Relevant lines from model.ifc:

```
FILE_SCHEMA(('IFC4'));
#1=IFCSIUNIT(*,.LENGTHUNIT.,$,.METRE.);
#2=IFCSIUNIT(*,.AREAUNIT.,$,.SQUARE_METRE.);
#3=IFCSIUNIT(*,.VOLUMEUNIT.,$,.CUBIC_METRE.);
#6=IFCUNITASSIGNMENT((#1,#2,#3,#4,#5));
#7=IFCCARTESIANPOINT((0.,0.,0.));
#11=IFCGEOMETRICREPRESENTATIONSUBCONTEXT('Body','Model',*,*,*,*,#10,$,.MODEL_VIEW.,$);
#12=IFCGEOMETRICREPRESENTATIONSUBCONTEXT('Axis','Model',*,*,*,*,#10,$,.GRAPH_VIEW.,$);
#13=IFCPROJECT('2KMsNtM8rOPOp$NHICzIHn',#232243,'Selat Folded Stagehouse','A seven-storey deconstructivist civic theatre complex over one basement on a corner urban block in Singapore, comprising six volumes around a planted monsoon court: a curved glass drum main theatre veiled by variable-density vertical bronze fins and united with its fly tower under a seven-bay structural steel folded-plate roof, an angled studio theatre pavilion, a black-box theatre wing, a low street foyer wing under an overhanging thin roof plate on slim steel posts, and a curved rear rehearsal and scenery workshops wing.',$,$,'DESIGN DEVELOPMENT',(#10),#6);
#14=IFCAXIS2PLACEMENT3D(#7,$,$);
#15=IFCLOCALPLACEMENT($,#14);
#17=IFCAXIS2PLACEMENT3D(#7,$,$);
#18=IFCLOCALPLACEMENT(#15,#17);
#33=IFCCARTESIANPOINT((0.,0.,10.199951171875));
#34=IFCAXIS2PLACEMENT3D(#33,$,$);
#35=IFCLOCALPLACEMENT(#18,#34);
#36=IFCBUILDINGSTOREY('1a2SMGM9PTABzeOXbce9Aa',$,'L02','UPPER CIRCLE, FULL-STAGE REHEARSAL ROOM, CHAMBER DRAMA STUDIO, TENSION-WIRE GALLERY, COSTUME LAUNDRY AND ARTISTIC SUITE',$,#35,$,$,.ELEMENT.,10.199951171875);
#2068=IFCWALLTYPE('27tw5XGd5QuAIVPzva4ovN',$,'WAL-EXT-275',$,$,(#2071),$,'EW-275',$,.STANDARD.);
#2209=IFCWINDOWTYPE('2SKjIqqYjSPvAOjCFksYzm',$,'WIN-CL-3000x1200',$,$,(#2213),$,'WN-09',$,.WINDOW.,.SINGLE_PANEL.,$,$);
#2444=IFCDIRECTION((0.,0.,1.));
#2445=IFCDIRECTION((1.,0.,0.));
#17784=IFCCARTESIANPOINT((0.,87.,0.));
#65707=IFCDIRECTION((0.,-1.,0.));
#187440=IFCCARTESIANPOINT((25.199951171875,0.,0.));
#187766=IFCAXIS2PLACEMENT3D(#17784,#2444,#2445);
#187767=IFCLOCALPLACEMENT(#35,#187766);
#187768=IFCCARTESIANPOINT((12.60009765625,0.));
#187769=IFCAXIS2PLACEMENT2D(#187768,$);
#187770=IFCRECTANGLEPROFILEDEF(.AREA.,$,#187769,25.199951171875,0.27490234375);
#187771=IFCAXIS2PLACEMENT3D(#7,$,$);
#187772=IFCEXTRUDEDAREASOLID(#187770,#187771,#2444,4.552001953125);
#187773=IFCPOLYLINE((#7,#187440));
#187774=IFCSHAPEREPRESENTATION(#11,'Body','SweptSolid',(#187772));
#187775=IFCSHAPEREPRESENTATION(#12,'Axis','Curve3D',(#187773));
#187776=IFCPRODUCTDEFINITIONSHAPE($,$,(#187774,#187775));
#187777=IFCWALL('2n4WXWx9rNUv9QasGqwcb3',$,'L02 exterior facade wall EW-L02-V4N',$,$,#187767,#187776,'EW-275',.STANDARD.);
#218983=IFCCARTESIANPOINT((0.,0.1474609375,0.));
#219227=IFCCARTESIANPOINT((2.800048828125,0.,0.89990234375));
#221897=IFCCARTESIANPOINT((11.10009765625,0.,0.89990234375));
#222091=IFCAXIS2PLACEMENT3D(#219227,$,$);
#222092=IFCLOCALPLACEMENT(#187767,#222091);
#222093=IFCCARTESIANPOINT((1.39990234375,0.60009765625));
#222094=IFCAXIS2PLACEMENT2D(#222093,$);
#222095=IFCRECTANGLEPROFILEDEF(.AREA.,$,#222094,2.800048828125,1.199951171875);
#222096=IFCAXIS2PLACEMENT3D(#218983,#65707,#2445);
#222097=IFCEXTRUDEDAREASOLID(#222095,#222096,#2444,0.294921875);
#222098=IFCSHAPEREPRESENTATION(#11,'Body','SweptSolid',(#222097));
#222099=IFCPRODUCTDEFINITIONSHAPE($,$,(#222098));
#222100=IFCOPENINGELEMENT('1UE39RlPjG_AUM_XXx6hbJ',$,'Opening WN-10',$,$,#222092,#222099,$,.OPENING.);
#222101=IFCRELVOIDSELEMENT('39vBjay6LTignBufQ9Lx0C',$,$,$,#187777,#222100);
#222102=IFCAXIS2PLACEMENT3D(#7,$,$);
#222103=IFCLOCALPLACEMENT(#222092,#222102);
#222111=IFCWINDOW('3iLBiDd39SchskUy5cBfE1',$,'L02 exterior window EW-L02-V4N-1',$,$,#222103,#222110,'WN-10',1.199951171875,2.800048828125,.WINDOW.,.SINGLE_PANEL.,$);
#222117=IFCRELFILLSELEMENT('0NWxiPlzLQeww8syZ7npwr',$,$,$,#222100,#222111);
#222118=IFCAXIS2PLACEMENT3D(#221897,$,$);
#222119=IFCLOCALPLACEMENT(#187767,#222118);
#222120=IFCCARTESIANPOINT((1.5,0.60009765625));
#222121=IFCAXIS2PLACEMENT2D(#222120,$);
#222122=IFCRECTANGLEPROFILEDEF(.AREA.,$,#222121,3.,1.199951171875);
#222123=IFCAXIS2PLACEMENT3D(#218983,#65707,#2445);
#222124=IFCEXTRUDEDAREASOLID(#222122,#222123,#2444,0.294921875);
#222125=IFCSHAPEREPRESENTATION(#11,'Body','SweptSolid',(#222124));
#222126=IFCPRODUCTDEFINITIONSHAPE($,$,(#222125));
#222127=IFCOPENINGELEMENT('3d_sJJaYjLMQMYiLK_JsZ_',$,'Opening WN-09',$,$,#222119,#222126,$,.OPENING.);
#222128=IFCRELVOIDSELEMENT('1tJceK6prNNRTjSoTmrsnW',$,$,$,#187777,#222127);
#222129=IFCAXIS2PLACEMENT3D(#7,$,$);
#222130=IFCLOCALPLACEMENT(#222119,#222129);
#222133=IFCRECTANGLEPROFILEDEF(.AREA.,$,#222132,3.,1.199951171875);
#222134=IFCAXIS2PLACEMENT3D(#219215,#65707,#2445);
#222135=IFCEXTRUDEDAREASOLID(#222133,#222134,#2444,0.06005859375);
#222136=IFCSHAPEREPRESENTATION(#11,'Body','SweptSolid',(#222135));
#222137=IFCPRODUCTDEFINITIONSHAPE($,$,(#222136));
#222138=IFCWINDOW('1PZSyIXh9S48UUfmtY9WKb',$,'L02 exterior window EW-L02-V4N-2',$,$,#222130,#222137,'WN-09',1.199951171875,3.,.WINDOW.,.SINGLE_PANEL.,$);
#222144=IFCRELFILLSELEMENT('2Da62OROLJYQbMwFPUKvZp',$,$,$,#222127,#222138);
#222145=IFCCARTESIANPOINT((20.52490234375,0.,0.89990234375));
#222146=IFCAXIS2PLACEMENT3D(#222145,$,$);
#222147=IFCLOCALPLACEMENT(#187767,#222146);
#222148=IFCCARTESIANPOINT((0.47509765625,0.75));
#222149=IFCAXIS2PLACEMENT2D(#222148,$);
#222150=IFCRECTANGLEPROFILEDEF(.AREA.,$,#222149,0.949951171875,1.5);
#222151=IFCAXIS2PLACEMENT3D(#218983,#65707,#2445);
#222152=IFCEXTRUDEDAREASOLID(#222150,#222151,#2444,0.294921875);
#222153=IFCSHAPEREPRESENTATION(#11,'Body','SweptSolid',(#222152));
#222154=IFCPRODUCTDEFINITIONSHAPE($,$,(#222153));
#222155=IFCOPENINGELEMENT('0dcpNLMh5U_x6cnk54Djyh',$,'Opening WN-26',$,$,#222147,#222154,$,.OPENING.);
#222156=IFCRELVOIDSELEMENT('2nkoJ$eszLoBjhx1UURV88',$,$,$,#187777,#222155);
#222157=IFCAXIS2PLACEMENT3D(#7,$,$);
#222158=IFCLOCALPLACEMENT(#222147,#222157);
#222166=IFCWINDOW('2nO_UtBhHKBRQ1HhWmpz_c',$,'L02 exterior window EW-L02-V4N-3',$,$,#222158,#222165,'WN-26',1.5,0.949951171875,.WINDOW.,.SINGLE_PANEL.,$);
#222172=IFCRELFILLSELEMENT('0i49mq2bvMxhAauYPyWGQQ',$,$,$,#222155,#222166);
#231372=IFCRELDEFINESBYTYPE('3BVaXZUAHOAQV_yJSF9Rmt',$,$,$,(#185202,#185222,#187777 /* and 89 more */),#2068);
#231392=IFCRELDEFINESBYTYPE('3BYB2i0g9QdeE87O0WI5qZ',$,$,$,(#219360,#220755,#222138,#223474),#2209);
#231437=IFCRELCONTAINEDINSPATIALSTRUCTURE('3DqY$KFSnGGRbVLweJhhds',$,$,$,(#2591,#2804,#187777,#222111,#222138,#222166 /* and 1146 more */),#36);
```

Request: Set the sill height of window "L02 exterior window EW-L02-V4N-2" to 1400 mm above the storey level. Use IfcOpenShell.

```python
import numpy as np
import ifcopenshell
import ifcopenshell.api.geometry
import ifcopenshell.geom
import ifcopenshell.util.element
import ifcopenshell.util.placement
import ifcopenshell.util.shape
import ifcopenshell.util.unit

model = ifcopenshell.open("model.ifc")
unit_scale = ifcopenshell.util.unit.calculate_unit_scale(model)

window = model.by_id(222138)
opening = window.FillsVoids[0].RelatingOpeningElement
storey = ifcopenshell.util.element.get_container(window, ifc_class="IfcBuildingStorey")
level = ifcopenshell.util.placement.get_local_placement(storey.ObjectPlacement)[2, 3]

# The opening's origin need not be at the sill, so measure its lowest point.
shape = ifcopenshell.geom.create_shape(ifcopenshell.geom.settings(), opening)
bottom = ifcopenshell.util.shape.get_shape_bottom_elevation(shape, shape.geometry) / unit_scale
dz = level + 1.4 / unit_scale - bottom

shift = np.array([0.0, 0.0, dz])
# The window is placed relative to its opening, so it follows when the opening moves.
matrix = ifcopenshell.util.placement.get_local_placement(opening.ObjectPlacement)
matrix[:3, 3] += shift
ifcopenshell.api.geometry.edit_object_placement(
    model, product=opening, matrix=matrix, is_si=False, should_transform_children=True
)

print(f"moved by {dz * unit_scale:+.3f} m")

model.write("model_updated.ifc")
```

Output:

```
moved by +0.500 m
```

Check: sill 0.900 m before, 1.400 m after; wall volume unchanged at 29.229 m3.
